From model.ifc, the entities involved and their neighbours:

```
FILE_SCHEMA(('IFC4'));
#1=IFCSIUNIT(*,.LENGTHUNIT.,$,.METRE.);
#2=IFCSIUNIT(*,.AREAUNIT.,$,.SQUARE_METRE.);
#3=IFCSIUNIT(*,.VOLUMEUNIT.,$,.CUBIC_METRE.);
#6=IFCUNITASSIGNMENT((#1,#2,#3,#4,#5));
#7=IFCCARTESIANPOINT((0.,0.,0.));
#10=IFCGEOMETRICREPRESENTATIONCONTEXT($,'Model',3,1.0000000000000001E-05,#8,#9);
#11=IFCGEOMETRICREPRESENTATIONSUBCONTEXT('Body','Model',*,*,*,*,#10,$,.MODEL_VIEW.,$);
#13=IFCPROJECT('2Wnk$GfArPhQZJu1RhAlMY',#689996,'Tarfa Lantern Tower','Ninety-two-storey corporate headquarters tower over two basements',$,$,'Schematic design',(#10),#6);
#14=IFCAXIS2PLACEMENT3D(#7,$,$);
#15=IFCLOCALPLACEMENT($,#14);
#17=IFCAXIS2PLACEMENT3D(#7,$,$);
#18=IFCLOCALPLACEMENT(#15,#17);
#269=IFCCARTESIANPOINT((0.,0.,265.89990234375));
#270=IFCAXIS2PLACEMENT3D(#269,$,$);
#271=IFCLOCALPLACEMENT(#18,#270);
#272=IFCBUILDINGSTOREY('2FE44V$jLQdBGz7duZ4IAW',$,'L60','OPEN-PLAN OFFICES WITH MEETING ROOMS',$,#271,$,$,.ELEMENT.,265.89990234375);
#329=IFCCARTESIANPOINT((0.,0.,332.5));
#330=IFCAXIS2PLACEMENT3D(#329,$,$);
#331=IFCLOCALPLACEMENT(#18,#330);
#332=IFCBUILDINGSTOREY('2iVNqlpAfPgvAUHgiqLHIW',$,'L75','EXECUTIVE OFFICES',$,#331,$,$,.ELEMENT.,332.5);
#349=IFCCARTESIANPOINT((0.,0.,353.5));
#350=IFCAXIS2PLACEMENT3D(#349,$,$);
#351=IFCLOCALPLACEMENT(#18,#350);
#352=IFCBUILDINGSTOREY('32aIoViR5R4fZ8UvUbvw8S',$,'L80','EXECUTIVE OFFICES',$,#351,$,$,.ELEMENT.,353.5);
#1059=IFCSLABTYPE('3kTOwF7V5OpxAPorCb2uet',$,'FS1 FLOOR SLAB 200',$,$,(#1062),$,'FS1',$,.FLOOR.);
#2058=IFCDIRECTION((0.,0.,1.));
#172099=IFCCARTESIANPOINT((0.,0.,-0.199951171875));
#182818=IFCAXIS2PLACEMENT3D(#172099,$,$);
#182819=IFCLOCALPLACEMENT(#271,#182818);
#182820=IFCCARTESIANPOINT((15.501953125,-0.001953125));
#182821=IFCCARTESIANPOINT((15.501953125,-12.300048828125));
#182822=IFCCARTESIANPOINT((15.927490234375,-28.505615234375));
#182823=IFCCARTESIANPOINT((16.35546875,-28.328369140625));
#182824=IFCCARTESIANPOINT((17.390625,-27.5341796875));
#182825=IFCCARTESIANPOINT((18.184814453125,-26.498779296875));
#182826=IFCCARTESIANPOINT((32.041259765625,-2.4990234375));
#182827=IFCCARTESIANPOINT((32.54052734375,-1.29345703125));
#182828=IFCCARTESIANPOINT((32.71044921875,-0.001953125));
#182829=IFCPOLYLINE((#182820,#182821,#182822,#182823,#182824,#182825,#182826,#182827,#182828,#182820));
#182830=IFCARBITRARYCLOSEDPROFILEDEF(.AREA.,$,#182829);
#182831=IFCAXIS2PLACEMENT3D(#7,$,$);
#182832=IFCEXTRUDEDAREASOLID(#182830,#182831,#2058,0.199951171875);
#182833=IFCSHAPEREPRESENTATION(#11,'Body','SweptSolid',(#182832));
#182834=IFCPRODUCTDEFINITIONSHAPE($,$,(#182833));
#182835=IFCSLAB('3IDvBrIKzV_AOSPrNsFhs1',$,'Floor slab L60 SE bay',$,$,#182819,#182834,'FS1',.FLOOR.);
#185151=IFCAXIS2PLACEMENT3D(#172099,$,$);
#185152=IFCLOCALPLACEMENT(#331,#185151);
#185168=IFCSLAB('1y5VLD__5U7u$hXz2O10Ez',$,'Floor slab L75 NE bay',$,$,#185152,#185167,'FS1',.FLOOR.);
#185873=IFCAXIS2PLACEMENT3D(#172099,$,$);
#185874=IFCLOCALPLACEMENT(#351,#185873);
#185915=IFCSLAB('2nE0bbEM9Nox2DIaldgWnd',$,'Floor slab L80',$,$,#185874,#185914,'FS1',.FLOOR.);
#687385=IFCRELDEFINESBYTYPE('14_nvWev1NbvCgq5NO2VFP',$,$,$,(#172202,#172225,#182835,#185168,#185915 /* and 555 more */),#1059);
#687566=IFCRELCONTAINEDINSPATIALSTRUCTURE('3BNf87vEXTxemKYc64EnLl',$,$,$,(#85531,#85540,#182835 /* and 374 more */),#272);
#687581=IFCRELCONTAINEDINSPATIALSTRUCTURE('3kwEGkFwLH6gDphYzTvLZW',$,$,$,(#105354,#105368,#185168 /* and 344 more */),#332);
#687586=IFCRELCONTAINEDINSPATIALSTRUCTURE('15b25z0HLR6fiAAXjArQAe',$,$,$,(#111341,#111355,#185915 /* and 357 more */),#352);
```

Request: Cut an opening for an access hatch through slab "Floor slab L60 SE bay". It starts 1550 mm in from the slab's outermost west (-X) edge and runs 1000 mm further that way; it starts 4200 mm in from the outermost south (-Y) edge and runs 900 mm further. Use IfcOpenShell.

```python
import numpy as np
import ifcopenshell
import ifcopenshell.api.feature
import ifcopenshell.api.geometry
import ifcopenshell.api.root
import ifcopenshell.geom
import ifcopenshell.util.placement
import ifcopenshell.util.representation
import ifcopenshell.util.shape
import ifcopenshell.util.unit

model = ifcopenshell.open("model.ifc")
unit_scale = ifcopenshell.util.unit.calculate_unit_scale(model)
settings = ifcopenshell.geom.settings()


def volume(element):
    """Net volume in cubic metres, openings subtracted."""
    shape = ifcopenshell.geom.create_shape(settings, element)
    return ifcopenshell.util.shape.get_volume(shape.geometry)


slab = model.by_id(182835)
before = volume(slab)

# Extent in the slab's own axes, in metres. The edges named are its -X and -Y sides.
slab_shape = ifcopenshell.geom.create_shape(settings, slab)
vertices = ifcopenshell.util.shape.get_vertices(slab_shape.geometry)
x_min, y_min, bottom = vertices.min(axis=0)
top = vertices[:, 2].max()

opening = ifcopenshell.api.root.create_entity(model, ifc_class="IfcOpeningElement", name="Access hatch opening", predefined_type="OPENING")
context = ifcopenshell.util.representation.get_context(model, "Model", "Body", "MODEL_VIEW")
width, depth = 1, 0.9
outline = [(0.0, 0.0), (width, 0.0), (width, depth), (0.0, depth), (0.0, 0.0)]
# Overshoot both faces by 50 mm so the cut is clean.
shape = ifcopenshell.api.geometry.add_slab_representation(
    model, context=context, depth=top - bottom + 0.1, polyline=outline
)
ifcopenshell.api.geometry.assign_representation(model, product=opening, representation=shape)

matrix = ifcopenshell.util.placement.get_local_placement(slab.ObjectPlacement)
matrix[:, 3] = matrix @ np.append(np.array([x_min + 1.55, y_min + 4.2, bottom - 0.05]) / unit_scale, 1.0)
ifcopenshell.api.geometry.edit_object_placement(model, product=opening, matrix=matrix, is_si=False)
ifcopenshell.api.feature.add_feature(model, feature=opening, element=slab)

after = volume(slab)

print(f"slab volume {before:.3f} -> {after:.3f} m3")

model.write("model_v2.ifc")
```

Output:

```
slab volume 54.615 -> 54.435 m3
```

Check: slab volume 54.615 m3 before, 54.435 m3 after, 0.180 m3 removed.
